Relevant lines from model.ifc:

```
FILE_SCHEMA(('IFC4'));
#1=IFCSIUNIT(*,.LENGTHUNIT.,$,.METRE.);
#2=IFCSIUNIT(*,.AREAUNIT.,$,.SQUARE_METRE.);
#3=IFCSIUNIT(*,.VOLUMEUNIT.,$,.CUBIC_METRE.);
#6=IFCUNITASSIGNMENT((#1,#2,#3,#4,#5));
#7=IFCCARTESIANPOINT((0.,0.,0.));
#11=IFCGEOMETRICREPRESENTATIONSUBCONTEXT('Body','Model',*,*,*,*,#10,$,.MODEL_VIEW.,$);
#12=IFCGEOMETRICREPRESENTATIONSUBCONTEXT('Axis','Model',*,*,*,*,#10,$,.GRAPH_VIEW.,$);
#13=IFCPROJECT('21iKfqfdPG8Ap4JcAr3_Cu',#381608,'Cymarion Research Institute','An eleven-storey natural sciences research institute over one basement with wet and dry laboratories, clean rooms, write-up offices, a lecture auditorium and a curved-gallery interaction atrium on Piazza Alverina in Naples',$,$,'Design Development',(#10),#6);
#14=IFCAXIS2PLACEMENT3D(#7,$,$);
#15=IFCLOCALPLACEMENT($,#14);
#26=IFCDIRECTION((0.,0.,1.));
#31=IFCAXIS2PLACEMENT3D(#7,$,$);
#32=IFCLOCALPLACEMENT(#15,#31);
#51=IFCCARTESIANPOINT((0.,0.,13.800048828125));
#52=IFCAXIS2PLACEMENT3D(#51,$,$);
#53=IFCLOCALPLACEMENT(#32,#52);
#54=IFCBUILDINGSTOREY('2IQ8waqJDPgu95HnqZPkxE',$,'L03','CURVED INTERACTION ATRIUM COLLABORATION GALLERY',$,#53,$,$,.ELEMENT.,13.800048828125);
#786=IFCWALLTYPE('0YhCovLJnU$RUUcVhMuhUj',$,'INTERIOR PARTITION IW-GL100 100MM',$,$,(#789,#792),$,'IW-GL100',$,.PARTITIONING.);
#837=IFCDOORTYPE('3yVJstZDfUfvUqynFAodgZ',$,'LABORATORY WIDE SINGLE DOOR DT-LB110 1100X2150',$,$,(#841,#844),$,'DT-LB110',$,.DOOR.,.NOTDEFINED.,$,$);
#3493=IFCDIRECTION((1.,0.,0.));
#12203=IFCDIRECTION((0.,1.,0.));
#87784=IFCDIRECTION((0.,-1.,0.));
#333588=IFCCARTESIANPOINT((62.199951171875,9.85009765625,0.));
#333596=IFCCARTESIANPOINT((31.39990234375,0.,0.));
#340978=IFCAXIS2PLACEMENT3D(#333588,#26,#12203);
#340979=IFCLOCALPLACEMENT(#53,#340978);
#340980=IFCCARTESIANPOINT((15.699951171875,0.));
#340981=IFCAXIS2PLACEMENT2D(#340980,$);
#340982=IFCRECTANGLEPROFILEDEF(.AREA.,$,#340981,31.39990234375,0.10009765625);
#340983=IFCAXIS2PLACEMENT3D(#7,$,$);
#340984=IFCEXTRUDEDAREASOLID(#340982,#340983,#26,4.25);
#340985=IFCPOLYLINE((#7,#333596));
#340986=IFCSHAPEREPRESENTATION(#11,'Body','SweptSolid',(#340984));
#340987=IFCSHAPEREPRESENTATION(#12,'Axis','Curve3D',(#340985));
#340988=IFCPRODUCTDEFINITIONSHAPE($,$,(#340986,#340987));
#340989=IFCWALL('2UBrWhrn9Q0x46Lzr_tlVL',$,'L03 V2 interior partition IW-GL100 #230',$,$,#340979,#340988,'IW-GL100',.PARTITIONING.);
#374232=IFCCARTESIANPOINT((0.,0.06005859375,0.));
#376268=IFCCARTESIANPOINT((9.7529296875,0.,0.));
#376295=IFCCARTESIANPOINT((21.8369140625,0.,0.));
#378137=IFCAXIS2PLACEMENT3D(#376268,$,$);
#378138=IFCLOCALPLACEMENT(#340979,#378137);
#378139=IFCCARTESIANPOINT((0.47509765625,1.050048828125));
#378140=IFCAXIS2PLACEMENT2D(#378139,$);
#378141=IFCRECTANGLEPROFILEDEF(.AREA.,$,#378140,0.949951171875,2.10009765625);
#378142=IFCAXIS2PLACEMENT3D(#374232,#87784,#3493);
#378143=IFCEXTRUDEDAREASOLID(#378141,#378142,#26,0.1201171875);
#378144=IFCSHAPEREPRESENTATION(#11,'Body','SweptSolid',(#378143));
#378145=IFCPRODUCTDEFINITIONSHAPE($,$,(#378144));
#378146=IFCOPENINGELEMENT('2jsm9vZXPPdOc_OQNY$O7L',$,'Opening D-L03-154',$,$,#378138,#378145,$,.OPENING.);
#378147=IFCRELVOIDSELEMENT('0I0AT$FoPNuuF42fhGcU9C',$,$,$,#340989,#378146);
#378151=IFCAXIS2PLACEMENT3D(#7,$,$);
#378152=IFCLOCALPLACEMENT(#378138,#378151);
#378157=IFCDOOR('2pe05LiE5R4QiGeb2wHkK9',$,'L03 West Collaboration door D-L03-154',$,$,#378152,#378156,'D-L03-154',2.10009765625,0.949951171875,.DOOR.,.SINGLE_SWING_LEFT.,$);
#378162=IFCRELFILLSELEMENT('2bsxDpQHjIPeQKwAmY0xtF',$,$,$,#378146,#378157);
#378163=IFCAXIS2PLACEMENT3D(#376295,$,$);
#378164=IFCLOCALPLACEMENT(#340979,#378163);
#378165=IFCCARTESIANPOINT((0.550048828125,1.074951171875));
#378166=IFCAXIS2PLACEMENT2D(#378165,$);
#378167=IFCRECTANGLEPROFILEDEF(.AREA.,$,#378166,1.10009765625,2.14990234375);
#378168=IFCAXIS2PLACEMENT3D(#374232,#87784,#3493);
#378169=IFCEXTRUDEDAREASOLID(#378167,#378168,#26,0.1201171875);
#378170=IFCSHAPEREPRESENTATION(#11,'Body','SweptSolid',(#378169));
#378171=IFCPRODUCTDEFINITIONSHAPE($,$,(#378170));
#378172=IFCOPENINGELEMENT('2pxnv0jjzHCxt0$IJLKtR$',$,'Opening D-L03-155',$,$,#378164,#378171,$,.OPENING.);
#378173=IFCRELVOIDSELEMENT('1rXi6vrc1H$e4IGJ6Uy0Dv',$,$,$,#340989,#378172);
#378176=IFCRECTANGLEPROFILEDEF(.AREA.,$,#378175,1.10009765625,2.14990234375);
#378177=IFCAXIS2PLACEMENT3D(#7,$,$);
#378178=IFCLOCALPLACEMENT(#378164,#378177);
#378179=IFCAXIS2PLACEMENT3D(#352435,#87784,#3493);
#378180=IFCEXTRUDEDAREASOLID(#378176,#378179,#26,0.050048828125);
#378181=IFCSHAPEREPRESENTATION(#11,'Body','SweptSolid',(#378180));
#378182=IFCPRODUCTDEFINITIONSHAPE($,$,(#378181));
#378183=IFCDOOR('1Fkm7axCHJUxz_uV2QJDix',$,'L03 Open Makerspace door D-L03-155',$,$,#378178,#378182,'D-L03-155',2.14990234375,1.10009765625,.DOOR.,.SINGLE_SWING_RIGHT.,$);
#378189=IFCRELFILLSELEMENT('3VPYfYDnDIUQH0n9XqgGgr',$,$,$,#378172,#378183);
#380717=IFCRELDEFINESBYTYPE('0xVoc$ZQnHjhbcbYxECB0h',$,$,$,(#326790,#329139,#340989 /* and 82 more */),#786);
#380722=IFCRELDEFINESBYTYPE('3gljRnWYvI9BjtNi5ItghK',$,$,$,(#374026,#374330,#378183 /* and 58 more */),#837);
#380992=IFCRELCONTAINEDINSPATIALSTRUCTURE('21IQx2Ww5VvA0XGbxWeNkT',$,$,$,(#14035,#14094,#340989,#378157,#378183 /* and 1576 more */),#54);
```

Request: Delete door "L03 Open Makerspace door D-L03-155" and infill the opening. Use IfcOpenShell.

```python
import ifcopenshell
import ifcopenshell.api.feature
import ifcopenshell.api.root
import ifcopenshell.geom
import ifcopenshell.util.shape

model = ifcopenshell.open("model.ifc")
settings = ifcopenshell.geom.settings()


def volume(element):
    """Net volume in cubic metres, openings subtracted."""
    shape = ifcopenshell.geom.create_shape(settings, element)
    return ifcopenshell.util.shape.get_volume(shape.geometry)


door = model.by_guid("1Fkm7axCHJUxz_uV2QJDix")
opening = door.FillsVoids[0].RelatingOpeningElement
wall = opening.VoidsElements[0].RelatingBuildingElement
before = volume(wall)

ifcopenshell.api.root.remove_product(model, product=door)
ifcopenshell.api.feature.remove_feature(model, feature=opening)

after = volume(wall)

print(f"wall volume {before:.3f} -> {after:.3f} m3")

model.write("model_edited.ifc")
```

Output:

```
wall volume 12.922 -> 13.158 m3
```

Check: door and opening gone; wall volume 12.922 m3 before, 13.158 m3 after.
